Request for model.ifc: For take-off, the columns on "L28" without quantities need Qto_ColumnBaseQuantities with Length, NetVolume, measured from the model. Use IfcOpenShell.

First a look at what the model holds.

```python
import ifcopenshell
import ifcopenshell.util.element
import ifcopenshell.util.unit

model = ifcopenshell.open("model.ifc")
print(model.schema)
for unit_type in ("LENGTHUNIT", "AREAUNIT", "VOLUMEUNIT"):
    print(unit_type, ifcopenshell.util.unit.calculate_unit_scale(model, unit_type))
storey = next(s for s in model.by_type("IfcBuildingStorey") if s.Name == "L28")
columns = [e for e in ifcopenshell.util.element.get_decomposition(storey) if e.is_a("IfcColumn")]
for e in sorted(columns, key=lambda e: e.id()):
    print(e.id(), e.is_a(), e.Name, list(ifcopenshell.util.element.get_psets(e, qtos_only=True)), sep=" | ")
```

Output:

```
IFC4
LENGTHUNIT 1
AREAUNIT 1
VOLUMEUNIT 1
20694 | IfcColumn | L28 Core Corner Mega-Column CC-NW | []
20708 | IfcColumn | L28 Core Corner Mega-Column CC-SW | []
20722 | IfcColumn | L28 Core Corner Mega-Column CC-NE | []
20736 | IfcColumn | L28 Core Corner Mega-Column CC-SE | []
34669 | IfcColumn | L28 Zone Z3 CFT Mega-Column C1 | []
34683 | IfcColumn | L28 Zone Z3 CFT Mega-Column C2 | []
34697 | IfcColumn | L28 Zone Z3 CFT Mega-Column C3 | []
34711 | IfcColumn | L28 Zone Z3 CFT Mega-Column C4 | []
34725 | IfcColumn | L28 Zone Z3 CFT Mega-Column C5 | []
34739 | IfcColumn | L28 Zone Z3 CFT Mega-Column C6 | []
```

```python
import ifcopenshell
import ifcopenshell.api.pset
import ifcopenshell.geom
import ifcopenshell.util.element
import ifcopenshell.util.shape
import ifcopenshell.util.unit

model = ifcopenshell.open("model.ifc")
unit_scale = ifcopenshell.util.unit.calculate_unit_scale(model)
volume_scale = ifcopenshell.util.unit.calculate_unit_scale(model, "VOLUMEUNIT")
settings = ifcopenshell.geom.settings()

storey = next(s for s in model.by_type("IfcBuildingStorey") if s.Name == "L28")
columns = [e for e in ifcopenshell.util.element.get_decomposition(storey) if e.is_a("IfcColumn")]

for e in sorted(columns, key=lambda e: e.id()):
    if ifcopenshell.util.element.get_psets(e, qtos_only=True, should_inherit=False):
        continue
    # Geometry comes back in metres, in the element's own axes.
    shape = ifcopenshell.geom.create_shape(settings, e)
    values = {
        "Length": ifcopenshell.util.shape.get_z(shape.geometry) / unit_scale,
        "NetVolume": ifcopenshell.util.shape.get_volume(shape.geometry) / volume_scale,
    }
    qto = ifcopenshell.api.pset.add_qto(model, product=e, name="Qto_ColumnBaseQuantities")
    ifcopenshell.api.pset.edit_qto(model, qto=qto, properties=values)
    print(e.id(), {k: round(v, 3) for k, v in values.items()})

model.write("model_edited.ifc")
```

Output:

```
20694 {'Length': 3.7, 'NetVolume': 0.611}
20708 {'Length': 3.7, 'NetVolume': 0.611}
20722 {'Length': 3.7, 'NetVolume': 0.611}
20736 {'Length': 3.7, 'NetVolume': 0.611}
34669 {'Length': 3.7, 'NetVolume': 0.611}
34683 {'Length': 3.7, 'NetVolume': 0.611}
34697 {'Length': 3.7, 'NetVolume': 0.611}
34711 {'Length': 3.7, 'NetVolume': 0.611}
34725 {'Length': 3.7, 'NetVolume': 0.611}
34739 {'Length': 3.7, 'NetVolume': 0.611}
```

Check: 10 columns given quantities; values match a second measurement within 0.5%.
